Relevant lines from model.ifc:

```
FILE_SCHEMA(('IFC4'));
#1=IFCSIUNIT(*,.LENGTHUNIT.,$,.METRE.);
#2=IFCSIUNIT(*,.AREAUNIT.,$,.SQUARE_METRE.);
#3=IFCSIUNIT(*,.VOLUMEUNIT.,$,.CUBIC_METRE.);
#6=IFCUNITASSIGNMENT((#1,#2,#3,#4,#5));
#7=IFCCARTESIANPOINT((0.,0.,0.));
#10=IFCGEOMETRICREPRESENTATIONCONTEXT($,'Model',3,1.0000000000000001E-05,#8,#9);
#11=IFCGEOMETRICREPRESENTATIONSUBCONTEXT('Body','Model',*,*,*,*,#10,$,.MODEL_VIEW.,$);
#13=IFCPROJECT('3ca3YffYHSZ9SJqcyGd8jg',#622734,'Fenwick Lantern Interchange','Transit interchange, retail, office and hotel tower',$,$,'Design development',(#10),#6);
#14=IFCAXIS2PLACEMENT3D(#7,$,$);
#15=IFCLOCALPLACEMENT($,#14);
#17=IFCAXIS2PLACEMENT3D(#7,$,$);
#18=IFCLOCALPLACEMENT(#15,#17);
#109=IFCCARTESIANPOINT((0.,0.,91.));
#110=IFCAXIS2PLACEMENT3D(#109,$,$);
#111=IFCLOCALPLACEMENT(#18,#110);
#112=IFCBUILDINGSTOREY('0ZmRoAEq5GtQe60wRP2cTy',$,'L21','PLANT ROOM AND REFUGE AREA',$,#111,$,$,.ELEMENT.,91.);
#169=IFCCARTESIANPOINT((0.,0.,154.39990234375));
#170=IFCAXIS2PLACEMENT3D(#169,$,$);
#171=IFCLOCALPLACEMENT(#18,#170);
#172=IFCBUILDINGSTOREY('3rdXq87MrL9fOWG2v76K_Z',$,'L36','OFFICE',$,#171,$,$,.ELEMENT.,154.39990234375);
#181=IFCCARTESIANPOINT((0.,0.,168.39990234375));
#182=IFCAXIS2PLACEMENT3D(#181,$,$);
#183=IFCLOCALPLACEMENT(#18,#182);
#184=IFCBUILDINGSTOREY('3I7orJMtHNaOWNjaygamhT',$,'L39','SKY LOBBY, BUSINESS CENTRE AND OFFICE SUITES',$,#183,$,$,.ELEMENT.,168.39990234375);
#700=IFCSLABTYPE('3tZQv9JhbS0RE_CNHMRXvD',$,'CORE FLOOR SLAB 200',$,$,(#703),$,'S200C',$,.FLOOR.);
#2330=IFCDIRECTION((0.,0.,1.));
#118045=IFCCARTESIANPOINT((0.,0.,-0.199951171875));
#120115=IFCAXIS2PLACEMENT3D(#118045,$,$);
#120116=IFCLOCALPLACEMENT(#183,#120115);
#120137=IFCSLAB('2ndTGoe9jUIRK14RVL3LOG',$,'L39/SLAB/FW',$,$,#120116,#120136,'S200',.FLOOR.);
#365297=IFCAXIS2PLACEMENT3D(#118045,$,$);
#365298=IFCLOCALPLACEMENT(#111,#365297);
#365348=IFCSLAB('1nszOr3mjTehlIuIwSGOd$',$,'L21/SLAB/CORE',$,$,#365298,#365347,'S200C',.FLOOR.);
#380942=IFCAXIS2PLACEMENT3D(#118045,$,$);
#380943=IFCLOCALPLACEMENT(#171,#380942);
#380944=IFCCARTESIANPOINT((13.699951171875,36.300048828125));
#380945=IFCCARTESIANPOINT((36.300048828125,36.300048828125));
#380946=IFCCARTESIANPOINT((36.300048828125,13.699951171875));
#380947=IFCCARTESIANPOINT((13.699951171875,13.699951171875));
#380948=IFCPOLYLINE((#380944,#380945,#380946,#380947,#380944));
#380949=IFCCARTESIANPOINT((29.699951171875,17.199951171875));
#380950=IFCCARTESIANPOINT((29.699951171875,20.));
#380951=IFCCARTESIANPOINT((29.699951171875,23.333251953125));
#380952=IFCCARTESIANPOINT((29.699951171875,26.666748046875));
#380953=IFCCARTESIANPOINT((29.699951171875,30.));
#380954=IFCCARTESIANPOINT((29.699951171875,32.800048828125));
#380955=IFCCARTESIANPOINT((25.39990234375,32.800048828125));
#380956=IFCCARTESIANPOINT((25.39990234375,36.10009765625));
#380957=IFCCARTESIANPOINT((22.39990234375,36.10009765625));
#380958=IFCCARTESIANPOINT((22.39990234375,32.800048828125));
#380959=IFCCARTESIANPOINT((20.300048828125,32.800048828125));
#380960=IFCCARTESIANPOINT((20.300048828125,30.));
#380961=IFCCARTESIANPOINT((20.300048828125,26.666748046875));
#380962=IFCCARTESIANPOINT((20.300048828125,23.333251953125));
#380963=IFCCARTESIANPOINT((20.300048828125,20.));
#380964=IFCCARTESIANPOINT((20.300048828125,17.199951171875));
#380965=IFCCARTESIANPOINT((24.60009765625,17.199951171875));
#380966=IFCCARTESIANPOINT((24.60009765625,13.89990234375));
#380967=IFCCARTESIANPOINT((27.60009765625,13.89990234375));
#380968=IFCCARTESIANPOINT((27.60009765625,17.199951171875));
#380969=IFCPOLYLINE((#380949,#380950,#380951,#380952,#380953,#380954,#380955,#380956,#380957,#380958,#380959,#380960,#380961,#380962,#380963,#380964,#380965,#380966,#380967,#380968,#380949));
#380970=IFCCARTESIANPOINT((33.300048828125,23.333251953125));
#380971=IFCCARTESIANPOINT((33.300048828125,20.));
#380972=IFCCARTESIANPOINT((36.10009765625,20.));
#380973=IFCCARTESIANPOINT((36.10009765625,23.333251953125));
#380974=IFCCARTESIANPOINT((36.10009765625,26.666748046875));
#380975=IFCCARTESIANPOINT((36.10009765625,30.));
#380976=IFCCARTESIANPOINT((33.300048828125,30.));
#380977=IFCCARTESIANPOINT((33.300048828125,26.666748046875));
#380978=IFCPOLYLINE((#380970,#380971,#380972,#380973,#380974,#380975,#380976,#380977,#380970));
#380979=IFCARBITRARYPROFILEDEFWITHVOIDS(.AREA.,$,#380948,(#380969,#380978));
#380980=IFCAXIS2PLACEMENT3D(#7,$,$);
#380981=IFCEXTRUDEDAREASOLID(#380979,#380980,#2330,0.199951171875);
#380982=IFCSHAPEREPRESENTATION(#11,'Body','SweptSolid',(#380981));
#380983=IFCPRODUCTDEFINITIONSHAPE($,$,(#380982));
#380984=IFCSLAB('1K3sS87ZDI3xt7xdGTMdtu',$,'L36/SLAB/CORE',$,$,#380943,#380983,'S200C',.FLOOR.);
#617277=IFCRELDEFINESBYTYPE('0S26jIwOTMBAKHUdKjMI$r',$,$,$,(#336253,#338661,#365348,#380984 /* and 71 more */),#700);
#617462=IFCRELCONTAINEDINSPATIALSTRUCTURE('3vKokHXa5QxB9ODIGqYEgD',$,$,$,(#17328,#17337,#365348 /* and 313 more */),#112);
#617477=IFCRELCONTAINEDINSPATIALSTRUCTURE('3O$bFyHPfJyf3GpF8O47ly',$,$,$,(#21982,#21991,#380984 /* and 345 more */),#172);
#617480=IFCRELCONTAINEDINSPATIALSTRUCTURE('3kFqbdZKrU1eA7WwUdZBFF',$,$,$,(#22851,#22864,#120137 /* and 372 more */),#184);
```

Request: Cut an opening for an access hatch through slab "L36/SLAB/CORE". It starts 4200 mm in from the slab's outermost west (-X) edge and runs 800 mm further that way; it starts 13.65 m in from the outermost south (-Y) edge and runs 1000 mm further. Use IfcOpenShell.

```python
import numpy as np
import ifcopenshell
import ifcopenshell.api.feature
import ifcopenshell.api.geometry
import ifcopenshell.api.root
import ifcopenshell.geom
import ifcopenshell.util.placement
import ifcopenshell.util.representation
import ifcopenshell.util.shape
import ifcopenshell.util.unit

model = ifcopenshell.open("model.ifc")
unit_scale = ifcopenshell.util.unit.calculate_unit_scale(model)
settings = ifcopenshell.geom.settings()


def volume(element):
    """Net volume in cubic metres, openings subtracted."""
    shape = ifcopenshell.geom.create_shape(settings, element)
    return ifcopenshell.util.shape.get_volume(shape.geometry)


slab = model.by_guid("1K3sS87ZDI3xt7xdGTMdtu")
before = volume(slab)

# Extent in the slab's own axes, in metres. The edges named are its -X and -Y sides.
slab_shape = ifcopenshell.geom.create_shape(settings, slab)
vertices = ifcopenshell.util.shape.get_vertices(slab_shape.geometry)
x_min, y_min, bottom = vertices.min(axis=0)
top = vertices[:, 2].max()

opening = ifcopenshell.api.root.create_entity(model, ifc_class="IfcOpeningElement", name="Access hatch opening", predefined_type="OPENING")
context = ifcopenshell.util.representation.get_context(model, "Model", "Body", "MODEL_VIEW")
width, depth = 0.8, 1
outline = [(0.0, 0.0), (width, 0.0), (width, depth), (0.0, depth), (0.0, 0.0)]
# Overshoot both faces by 50 mm so the cut is clean.
shape = ifcopenshell.api.geometry.add_slab_representation(
    model, context=context, depth=top - bottom + 0.1, polyline=outline
)
ifcopenshell.api.geometry.assign_representation(model, product=opening, representation=shape)

matrix = ifcopenshell.util.placement.get_local_placement(slab.ObjectPlacement)
matrix[:, 3] = matrix @ np.append(np.array([x_min + 4.2, y_min + 13.65, bottom - 0.05]) / unit_scale, 1.0)
ifcopenshell.api.geometry.edit_object_placement(model, product=opening, matrix=matrix, is_si=False)
ifcopenshell.api.feature.add_feature(model, feature=opening, element=slab)

after = volume(slab)

print(f"slab volume {before:.3f} -> {after:.3f} m3")

model.write("model_updated.ifc")
```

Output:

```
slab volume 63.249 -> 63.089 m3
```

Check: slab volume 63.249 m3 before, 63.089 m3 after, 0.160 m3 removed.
